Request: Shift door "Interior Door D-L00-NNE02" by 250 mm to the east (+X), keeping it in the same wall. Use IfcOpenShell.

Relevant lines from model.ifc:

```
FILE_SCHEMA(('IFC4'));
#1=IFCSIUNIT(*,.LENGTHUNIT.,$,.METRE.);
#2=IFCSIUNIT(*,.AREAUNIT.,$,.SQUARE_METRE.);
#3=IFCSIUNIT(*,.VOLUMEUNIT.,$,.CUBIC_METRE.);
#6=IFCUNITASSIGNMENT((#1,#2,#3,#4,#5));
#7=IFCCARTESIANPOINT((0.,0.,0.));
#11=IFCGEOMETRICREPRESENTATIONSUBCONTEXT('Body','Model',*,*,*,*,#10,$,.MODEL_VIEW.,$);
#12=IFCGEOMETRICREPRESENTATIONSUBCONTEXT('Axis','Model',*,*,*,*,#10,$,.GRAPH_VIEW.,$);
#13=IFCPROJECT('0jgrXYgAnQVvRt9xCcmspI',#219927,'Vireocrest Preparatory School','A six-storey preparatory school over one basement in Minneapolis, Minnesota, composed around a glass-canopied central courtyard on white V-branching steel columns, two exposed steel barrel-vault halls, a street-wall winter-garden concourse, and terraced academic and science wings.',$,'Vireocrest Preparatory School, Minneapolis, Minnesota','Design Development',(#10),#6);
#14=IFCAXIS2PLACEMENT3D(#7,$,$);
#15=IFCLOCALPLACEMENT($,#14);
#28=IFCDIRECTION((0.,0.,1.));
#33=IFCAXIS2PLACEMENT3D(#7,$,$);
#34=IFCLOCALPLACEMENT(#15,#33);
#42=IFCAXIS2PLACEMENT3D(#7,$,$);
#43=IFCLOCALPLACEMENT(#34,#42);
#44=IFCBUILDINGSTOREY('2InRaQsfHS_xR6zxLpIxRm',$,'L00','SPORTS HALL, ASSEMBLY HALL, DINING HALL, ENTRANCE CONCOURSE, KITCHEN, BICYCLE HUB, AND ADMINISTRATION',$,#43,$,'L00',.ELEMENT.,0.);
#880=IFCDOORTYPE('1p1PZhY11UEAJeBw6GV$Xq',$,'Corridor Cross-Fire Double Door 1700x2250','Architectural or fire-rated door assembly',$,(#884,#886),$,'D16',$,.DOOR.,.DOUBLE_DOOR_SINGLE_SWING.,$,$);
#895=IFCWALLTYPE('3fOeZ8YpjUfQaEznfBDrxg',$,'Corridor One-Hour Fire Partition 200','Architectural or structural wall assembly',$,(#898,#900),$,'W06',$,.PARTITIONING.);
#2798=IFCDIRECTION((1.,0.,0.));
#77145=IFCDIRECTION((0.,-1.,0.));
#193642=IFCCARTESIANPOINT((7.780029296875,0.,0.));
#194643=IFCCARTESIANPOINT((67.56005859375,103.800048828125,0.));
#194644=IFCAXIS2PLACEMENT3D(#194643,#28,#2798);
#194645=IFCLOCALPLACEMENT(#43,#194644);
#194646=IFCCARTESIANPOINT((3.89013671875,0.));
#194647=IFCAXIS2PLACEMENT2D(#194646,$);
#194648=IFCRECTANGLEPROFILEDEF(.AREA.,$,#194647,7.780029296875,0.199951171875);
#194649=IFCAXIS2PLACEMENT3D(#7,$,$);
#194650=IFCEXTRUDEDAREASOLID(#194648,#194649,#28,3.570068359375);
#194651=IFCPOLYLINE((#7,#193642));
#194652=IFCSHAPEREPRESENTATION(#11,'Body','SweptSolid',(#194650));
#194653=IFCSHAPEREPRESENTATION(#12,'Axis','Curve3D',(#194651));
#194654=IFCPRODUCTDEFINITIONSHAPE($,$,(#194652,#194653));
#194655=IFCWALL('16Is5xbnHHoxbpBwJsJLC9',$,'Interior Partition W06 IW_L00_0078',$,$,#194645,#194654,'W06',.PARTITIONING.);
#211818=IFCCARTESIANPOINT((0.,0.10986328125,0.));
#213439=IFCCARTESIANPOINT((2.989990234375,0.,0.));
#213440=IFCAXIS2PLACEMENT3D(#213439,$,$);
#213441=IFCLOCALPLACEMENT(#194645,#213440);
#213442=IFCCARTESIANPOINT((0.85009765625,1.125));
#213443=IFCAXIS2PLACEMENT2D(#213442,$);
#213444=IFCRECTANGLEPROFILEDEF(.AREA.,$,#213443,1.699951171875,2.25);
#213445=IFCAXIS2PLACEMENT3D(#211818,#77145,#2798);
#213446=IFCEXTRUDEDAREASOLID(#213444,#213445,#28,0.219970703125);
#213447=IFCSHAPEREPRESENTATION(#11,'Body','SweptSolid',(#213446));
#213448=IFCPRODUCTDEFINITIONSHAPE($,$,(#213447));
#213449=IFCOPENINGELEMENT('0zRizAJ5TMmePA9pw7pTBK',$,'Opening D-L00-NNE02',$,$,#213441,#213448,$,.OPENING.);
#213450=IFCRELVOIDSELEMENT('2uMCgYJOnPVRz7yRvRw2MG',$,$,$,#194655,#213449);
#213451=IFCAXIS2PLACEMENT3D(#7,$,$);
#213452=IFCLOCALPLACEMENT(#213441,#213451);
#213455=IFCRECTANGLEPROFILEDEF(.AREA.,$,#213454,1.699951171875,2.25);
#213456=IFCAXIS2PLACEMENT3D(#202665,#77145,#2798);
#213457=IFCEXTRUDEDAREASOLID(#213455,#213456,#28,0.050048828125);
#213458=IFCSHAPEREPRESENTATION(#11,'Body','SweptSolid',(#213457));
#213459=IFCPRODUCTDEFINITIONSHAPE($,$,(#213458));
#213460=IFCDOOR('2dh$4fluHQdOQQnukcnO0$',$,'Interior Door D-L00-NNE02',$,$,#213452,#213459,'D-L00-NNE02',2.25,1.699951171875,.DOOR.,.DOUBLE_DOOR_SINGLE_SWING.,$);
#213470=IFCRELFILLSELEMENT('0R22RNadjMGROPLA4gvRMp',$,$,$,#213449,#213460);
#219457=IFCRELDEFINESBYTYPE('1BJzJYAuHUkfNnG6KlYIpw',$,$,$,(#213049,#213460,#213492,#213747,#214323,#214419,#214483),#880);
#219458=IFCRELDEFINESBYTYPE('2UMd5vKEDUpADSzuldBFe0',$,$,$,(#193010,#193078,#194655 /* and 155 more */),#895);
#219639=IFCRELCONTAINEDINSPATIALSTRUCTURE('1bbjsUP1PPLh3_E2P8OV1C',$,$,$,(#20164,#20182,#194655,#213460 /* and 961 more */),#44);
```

```python
import ifcopenshell
import ifcopenshell.api.geometry
import ifcopenshell.util.placement
import ifcopenshell.util.unit

model = ifcopenshell.open("model.ifc")
unit_scale = ifcopenshell.util.unit.calculate_unit_scale(model)

door = model.by_guid("2dh$4fluHQdOQQnukcnO0$")
opening = door.FillsVoids[0].RelatingOpeningElement
wall = opening.VoidsElements[0].RelatingBuildingElement

wall_matrix = ifcopenshell.util.placement.get_local_placement(wall.ObjectPlacement)
shift = wall_matrix[:3, 0] * 0.25 / unit_scale
before = ifcopenshell.util.placement.get_local_placement(door.ObjectPlacement)[:3, 3].copy()

# The door is placed relative to its opening, so it follows when the opening moves.
matrix = ifcopenshell.util.placement.get_local_placement(opening.ObjectPlacement)
matrix[:3, 3] += shift
ifcopenshell.api.geometry.edit_object_placement(
    model, product=opening, matrix=matrix, is_si=False, should_transform_children=True
)

after = ifcopenshell.util.placement.get_local_placement(door.ObjectPlacement)[:3, 3]
print("door moved by", (after - before).round(3) + 0.0)

model.write("model-out.ifc")
```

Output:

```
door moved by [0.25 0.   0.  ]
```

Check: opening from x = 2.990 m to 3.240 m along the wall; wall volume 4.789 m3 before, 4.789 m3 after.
